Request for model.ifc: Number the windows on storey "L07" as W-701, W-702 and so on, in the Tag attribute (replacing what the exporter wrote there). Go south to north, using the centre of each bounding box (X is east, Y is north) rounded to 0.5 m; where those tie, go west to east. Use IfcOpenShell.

First a look at what the model holds.

```python
import ifcopenshell
import ifcopenshell.util.element
import ifcopenshell.util.placement

model = ifcopenshell.open("model.ifc")
print(model.schema)
storey = next(s for s in model.by_type("IfcBuildingStorey") if s.Name == "L07")
windows = [e for e in ifcopenshell.util.element.get_decomposition(storey) if e.is_a("IfcWindow")]
for e in sorted(windows, key=lambda e: e.id()):
    origin = ifcopenshell.util.placement.get_local_placement(e.ObjectPlacement)[:3, 3]
    print(e.id(), e.Tag, e.Name, origin.round(2) + 0.0, sep=" | ")
```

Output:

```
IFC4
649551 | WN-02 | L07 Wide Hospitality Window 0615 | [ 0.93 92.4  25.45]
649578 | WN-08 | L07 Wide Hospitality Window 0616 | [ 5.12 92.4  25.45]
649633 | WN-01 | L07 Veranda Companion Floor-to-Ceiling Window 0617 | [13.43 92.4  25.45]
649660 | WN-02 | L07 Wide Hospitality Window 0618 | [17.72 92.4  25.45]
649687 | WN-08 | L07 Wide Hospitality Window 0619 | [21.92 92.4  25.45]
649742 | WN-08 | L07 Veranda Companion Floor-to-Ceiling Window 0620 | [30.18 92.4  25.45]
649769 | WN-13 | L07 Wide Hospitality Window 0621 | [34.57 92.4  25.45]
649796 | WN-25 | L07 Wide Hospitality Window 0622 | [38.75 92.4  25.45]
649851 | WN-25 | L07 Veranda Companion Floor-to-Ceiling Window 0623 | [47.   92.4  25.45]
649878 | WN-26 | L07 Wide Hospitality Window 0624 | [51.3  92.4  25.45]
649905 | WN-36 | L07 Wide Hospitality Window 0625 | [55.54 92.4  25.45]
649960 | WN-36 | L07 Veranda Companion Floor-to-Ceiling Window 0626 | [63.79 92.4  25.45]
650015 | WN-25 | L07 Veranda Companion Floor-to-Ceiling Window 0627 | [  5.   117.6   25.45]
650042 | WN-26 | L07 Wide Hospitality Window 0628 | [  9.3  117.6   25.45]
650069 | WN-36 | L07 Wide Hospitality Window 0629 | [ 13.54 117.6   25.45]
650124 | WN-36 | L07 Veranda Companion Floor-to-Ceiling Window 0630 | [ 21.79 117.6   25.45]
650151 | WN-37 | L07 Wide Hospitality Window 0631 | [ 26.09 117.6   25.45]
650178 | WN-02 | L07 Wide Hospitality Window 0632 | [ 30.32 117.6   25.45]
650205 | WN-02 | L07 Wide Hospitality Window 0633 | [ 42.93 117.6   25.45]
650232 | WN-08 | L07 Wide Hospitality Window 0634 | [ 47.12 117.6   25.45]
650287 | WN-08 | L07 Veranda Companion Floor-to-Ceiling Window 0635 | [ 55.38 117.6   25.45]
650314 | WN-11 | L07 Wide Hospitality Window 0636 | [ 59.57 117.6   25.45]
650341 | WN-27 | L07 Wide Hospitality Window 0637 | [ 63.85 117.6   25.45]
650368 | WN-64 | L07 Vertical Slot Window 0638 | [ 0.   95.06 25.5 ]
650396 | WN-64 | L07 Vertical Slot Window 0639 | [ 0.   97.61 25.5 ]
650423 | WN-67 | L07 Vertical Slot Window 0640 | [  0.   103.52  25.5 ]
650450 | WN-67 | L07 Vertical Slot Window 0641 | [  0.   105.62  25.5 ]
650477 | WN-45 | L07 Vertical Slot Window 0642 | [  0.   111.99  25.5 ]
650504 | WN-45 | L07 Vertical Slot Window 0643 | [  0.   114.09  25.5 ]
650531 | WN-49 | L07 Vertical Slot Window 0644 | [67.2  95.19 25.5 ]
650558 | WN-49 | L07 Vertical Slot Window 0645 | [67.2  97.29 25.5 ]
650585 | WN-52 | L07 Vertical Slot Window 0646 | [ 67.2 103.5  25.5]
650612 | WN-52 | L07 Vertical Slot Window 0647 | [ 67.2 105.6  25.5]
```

```python
import ifcopenshell
import ifcopenshell.geom
import ifcopenshell.util.element
import ifcopenshell.util.shape

model = ifcopenshell.open("model.ifc")
settings = ifcopenshell.geom.settings()
settings.set("use-world-coords", True)


def centre(element):
    shape = ifcopenshell.geom.create_shape(settings, element)
    return ifcopenshell.util.shape.get_bbox_centroid(shape.geometry)


storey = next(s for s in model.by_type("IfcBuildingStorey") if s.Name == "L07")
windows = [e for e in ifcopenshell.util.element.get_decomposition(storey) if e.is_a("IfcWindow")]

# Insertion points can sit at a corner or the storey origin, so sort by the geometry (in metres).
centres = {e: centre(e) for e in windows}
windows.sort(key=lambda e: (round(centres[e][1] / 0.5), centres[e][0]))

for i, e in enumerate(windows, start=1):
    number = f"W-7{i:02d}"
    e.Tag = number
    print(e.id(), number)

model.write("model_v2.ifc")
```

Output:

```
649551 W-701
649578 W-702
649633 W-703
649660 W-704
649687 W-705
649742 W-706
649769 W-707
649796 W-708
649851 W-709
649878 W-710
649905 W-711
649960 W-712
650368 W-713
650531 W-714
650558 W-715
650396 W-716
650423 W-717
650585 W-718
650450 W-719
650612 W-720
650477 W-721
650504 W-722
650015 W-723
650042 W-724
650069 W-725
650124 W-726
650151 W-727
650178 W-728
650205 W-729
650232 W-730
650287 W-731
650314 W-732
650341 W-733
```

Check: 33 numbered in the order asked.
